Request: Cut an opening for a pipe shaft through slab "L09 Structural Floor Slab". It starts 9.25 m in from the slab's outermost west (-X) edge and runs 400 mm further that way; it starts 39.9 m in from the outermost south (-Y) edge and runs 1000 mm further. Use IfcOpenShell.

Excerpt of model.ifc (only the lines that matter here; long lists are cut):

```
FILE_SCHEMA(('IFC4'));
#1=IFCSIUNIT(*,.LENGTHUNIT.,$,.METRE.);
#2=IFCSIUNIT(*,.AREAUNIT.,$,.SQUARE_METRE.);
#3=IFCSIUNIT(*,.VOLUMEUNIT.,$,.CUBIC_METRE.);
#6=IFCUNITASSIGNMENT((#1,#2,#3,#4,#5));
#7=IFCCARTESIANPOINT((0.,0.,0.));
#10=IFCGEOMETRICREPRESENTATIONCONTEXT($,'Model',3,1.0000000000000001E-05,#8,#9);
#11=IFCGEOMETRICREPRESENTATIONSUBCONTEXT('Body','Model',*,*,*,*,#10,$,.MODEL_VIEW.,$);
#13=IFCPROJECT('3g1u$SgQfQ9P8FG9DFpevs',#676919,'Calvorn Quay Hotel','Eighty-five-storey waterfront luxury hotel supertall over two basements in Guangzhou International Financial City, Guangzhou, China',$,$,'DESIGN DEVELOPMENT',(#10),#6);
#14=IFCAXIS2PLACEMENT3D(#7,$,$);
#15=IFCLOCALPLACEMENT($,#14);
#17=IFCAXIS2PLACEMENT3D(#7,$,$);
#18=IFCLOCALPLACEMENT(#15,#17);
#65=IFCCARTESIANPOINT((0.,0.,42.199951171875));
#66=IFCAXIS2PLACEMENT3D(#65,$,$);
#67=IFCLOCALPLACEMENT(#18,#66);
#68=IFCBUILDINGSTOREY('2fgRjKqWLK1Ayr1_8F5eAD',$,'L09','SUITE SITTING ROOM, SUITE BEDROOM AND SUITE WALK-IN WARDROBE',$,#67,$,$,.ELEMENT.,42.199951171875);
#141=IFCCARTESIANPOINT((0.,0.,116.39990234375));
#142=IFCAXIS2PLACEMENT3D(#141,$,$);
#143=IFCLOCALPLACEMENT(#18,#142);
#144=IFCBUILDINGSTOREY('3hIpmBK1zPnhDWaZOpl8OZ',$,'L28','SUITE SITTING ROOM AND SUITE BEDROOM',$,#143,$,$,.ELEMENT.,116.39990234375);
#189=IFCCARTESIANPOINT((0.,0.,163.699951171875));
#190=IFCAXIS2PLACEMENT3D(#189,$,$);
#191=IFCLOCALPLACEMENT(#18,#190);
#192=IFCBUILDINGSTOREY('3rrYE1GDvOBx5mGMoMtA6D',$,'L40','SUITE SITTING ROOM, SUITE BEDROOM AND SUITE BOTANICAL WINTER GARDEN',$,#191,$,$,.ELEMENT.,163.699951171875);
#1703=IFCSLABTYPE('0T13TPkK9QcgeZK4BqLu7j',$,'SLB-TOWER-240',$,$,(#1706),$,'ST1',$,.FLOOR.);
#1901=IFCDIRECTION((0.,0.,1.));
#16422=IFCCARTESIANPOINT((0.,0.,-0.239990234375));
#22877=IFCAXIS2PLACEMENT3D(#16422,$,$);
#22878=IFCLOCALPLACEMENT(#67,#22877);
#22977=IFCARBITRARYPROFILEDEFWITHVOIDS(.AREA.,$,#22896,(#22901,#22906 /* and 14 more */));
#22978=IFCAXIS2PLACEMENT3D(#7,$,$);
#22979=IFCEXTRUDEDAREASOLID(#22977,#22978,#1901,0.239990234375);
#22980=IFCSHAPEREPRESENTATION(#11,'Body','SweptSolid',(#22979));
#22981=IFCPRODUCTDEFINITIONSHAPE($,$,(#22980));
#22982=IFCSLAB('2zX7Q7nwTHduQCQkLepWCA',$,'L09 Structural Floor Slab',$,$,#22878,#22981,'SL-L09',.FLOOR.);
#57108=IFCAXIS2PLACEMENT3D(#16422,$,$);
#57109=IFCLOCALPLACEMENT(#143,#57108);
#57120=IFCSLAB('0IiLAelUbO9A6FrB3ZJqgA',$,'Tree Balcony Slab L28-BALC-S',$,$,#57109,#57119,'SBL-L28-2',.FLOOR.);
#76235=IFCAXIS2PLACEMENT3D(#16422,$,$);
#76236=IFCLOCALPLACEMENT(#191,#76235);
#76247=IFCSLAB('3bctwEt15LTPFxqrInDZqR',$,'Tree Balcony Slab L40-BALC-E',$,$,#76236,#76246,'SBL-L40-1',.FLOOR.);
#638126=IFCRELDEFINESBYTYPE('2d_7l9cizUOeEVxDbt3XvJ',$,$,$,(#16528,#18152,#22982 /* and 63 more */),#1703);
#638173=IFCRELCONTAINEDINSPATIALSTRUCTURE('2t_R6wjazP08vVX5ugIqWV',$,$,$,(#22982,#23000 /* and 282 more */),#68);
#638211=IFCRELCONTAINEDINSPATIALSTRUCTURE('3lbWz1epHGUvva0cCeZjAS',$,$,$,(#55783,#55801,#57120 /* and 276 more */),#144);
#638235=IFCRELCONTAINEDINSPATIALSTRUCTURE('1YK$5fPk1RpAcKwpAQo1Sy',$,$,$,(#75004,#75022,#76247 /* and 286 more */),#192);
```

```python
import numpy as np
import ifcopenshell
import ifcopenshell.api.feature
import ifcopenshell.api.geometry
import ifcopenshell.api.root
import ifcopenshell.geom
import ifcopenshell.util.placement
import ifcopenshell.util.representation
import ifcopenshell.util.shape
import ifcopenshell.util.unit

model = ifcopenshell.open("model.ifc")
unit_scale = ifcopenshell.util.unit.calculate_unit_scale(model)
settings = ifcopenshell.geom.settings()


def volume(element):
    """Net volume in cubic metres, openings subtracted."""
    shape = ifcopenshell.geom.create_shape(settings, element)
    return ifcopenshell.util.shape.get_volume(shape.geometry)


slab = model.by_id(22982)
before = volume(slab)

# Extent in the slab's own axes, in metres. The edges named are its -X and -Y sides.
slab_shape = ifcopenshell.geom.create_shape(settings, slab)
vertices = ifcopenshell.util.shape.get_vertices(slab_shape.geometry)
x_min, y_min, bottom = vertices.min(axis=0)
top = vertices[:, 2].max()

opening = ifcopenshell.api.root.create_entity(model, ifc_class="IfcOpeningElement", name="Pipe shaft opening", predefined_type="OPENING")
context = ifcopenshell.util.representation.get_context(model, "Model", "Body", "MODEL_VIEW")
width, depth = 0.4, 1
outline = [(0.0, 0.0), (width, 0.0), (width, depth), (0.0, depth), (0.0, 0.0)]
# Overshoot both faces by 50 mm so the cut is clean.
shape = ifcopenshell.api.geometry.add_slab_representation(
    model, context=context, depth=top - bottom + 0.1, polyline=outline
)
ifcopenshell.api.geometry.assign_representation(model, product=opening, representation=shape)

matrix = ifcopenshell.util.placement.get_local_placement(slab.ObjectPlacement)
matrix[:, 3] = matrix @ np.append(np.array([x_min + 9.25, y_min + 39.9, bottom - 0.05]) / unit_scale, 1.0)
ifcopenshell.api.geometry.edit_object_placement(model, product=opening, matrix=matrix, is_si=False)
ifcopenshell.api.feature.add_feature(model, feature=opening, element=slab)

after = volume(slab)

print(f"slab volume {before:.3f} -> {after:.3f} m3")

model.write("model_edited.ifc")
```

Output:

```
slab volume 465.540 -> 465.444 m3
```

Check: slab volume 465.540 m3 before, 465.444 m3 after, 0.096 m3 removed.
